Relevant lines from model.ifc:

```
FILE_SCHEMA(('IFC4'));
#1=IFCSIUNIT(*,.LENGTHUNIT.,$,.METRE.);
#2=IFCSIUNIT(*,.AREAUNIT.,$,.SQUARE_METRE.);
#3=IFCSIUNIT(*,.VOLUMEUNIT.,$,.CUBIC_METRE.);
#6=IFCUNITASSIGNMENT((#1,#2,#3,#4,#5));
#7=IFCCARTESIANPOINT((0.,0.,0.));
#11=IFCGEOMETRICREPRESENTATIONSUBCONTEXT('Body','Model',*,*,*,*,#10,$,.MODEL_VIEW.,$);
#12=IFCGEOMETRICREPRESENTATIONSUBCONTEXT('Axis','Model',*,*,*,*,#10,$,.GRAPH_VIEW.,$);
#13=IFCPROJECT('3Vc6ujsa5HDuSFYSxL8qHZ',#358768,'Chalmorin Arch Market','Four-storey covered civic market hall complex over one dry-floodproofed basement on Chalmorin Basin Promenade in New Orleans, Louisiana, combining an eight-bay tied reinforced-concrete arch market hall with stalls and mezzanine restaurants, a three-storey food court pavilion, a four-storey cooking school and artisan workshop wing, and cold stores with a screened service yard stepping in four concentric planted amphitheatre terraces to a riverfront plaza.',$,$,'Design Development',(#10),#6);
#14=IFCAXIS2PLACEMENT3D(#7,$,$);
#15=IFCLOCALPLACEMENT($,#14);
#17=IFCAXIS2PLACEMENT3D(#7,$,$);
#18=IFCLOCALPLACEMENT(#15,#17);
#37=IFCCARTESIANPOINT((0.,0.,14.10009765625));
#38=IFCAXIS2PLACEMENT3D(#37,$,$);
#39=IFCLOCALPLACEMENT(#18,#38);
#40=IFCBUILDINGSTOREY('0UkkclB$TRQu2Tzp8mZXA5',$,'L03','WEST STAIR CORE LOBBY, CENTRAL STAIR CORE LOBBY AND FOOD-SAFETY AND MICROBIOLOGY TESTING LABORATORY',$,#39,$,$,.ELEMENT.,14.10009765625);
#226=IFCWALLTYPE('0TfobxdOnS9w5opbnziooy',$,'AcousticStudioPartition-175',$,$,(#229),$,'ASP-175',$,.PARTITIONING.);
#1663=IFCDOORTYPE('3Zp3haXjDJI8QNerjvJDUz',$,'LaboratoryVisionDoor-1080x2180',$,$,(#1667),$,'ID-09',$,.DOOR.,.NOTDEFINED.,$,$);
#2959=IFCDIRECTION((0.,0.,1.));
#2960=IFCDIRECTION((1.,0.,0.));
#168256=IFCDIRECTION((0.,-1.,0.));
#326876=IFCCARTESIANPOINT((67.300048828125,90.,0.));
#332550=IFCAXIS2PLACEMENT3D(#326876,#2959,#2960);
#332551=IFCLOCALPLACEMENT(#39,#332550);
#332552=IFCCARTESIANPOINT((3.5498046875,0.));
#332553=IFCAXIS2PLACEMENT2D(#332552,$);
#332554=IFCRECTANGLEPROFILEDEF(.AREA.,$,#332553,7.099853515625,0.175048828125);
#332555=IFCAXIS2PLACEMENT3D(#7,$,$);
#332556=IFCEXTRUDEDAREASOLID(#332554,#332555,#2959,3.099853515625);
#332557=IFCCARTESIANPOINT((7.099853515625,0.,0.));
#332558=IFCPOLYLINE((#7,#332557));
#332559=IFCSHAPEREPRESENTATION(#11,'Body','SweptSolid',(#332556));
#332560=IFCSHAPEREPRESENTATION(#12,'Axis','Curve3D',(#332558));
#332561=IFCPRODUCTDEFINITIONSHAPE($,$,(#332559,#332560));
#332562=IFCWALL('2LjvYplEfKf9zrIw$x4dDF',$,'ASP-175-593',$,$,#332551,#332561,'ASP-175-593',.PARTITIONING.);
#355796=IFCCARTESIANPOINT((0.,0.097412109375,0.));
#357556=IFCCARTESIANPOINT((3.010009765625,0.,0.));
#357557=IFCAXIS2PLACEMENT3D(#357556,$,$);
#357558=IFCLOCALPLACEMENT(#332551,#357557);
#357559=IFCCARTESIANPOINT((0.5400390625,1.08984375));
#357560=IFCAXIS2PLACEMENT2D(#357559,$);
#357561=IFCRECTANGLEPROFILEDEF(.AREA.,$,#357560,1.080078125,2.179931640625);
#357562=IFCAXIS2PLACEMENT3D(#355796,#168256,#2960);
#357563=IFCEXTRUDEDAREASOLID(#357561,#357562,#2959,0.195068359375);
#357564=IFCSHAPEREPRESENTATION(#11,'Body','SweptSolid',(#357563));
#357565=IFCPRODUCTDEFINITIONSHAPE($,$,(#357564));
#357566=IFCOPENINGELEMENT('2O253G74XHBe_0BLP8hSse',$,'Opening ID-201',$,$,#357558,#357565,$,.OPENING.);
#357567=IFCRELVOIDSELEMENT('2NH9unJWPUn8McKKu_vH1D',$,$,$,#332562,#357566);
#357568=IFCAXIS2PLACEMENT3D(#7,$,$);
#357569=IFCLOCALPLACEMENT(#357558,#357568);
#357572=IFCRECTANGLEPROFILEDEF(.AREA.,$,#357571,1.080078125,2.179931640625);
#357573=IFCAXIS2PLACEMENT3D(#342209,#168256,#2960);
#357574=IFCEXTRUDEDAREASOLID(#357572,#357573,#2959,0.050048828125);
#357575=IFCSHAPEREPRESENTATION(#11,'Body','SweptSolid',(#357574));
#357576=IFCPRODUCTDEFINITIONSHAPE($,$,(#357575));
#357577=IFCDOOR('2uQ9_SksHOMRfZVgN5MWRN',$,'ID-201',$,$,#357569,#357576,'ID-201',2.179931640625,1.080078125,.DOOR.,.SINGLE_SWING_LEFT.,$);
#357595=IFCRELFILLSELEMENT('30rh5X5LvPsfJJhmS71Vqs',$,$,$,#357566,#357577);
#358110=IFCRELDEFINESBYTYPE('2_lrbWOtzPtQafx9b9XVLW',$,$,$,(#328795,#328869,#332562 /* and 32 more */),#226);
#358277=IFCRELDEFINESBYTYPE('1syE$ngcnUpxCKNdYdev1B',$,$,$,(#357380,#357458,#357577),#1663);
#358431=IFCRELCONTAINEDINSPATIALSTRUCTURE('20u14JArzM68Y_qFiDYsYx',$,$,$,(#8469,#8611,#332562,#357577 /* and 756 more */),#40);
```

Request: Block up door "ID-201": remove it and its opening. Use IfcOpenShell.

```python
import ifcopenshell
import ifcopenshell.api.feature
import ifcopenshell.api.root
import ifcopenshell.geom
import ifcopenshell.util.shape

model = ifcopenshell.open("model.ifc")
settings = ifcopenshell.geom.settings()


def volume(element):
    """Net volume in cubic metres, openings subtracted."""
    shape = ifcopenshell.geom.create_shape(settings, element)
    return ifcopenshell.util.shape.get_volume(shape.geometry)


door = model.by_id(357577)
opening = door.FillsVoids[0].RelatingOpeningElement
wall = opening.VoidsElements[0].RelatingBuildingElement
before = volume(wall)

ifcopenshell.api.root.remove_product(model, product=door)
ifcopenshell.api.feature.remove_feature(model, feature=opening)

after = volume(wall)

print(f"wall volume {before:.3f} -> {after:.3f} m3")

model.write("model_updated.ifc")
```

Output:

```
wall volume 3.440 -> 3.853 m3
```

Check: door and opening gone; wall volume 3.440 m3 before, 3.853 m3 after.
